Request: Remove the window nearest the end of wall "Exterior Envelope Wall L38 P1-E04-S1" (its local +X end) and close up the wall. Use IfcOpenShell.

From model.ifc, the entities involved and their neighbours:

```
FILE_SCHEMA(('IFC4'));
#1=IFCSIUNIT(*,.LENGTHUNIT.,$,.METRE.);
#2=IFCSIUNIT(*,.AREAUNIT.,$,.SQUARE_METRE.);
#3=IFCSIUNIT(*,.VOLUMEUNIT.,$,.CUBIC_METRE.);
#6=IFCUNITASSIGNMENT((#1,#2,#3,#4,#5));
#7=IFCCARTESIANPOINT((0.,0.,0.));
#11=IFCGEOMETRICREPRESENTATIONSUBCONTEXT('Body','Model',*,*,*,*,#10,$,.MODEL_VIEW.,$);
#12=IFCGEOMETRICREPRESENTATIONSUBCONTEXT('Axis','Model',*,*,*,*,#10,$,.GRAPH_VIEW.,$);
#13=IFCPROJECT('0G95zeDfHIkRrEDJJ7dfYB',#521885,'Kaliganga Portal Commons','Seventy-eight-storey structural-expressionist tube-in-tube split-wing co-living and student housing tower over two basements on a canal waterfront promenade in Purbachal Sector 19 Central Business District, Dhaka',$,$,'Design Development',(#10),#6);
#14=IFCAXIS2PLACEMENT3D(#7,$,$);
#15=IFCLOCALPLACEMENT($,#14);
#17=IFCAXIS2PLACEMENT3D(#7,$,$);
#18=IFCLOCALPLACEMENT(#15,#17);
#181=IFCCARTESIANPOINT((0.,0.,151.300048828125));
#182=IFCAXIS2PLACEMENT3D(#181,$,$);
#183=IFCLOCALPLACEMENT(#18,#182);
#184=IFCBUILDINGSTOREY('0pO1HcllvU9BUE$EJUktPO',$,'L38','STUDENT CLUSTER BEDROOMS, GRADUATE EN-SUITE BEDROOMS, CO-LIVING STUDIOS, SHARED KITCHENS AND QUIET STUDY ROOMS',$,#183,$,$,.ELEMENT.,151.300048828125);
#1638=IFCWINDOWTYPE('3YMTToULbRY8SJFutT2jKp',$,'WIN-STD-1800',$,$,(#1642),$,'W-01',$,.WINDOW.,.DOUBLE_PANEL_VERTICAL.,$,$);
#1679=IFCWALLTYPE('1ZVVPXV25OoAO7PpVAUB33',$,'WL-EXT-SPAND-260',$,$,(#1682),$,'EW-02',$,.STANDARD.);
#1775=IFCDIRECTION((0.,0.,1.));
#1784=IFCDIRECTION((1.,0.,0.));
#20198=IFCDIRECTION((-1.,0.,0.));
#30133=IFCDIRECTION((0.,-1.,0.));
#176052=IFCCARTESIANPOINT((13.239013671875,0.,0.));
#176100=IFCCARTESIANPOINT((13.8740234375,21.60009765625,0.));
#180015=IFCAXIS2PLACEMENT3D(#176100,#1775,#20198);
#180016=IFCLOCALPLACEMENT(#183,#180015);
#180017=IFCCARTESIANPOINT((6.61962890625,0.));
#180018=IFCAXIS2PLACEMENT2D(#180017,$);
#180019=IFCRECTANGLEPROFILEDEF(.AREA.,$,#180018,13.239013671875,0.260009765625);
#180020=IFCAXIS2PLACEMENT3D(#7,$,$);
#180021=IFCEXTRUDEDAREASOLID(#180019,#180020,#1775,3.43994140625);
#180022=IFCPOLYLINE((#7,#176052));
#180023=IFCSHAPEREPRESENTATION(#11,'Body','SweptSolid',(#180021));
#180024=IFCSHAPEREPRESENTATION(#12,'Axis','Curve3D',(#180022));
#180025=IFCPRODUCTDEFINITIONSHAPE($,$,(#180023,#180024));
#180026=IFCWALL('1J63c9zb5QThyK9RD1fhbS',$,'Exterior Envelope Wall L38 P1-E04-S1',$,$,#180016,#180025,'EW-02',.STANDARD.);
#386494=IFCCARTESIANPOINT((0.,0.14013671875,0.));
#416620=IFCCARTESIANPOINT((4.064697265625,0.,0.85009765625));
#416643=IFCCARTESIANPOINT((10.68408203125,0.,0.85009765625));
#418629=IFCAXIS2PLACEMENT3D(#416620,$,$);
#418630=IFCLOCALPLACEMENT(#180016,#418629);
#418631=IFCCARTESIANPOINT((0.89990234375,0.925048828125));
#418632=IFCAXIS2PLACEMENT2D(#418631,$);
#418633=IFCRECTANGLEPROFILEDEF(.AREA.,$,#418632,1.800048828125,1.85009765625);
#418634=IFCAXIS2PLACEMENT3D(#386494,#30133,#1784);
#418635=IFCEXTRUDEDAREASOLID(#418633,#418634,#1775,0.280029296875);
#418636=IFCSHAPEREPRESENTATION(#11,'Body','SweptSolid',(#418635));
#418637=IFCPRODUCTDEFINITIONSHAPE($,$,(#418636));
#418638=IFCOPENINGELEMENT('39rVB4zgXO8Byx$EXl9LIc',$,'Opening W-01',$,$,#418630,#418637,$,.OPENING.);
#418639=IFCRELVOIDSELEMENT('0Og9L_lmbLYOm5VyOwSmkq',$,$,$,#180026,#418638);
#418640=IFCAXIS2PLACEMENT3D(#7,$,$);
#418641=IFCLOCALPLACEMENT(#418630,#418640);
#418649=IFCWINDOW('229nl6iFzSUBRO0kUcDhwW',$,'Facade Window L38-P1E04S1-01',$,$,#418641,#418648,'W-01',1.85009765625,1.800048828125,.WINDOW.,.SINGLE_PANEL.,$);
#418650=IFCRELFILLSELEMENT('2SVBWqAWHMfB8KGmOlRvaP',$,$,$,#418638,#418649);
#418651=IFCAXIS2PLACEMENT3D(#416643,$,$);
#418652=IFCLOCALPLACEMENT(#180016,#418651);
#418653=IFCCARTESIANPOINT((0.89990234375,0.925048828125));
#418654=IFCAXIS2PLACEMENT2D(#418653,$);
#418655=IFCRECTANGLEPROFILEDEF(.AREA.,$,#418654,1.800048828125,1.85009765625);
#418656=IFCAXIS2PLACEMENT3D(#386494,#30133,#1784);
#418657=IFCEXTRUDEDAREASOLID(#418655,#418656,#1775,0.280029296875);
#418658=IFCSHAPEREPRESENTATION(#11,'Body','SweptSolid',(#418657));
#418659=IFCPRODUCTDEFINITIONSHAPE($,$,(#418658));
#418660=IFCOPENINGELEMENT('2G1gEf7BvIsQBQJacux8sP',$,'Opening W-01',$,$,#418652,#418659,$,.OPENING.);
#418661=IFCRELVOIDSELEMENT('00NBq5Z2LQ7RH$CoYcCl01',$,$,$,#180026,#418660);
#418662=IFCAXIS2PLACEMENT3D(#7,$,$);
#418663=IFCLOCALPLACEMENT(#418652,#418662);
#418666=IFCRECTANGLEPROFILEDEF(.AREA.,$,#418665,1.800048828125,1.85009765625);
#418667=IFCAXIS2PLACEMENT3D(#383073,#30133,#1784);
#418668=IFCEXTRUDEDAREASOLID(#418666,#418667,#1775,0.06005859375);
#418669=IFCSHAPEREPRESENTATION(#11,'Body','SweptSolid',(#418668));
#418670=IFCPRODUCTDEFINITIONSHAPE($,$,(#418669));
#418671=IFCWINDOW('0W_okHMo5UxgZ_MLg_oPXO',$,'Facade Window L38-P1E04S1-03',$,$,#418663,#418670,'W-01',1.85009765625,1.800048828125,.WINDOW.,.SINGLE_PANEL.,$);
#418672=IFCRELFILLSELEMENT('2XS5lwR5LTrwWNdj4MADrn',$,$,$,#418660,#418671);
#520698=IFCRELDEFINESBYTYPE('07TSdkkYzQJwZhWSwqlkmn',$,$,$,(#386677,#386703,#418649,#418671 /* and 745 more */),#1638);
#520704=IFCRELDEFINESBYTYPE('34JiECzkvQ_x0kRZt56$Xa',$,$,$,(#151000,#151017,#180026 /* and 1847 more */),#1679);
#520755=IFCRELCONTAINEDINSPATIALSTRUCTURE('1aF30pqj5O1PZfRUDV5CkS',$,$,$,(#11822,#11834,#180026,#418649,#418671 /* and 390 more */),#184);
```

```python
import ifcopenshell
import ifcopenshell.api.feature
import ifcopenshell.api.root
import ifcopenshell.geom
import ifcopenshell.util.shape

model = ifcopenshell.open("model.ifc")
settings = ifcopenshell.geom.settings()


def volume(element):
    """Net volume in cubic metres, openings subtracted."""
    shape = ifcopenshell.geom.create_shape(settings, element)
    return ifcopenshell.util.shape.get_volume(shape.geometry)


window = model.by_id(418671)
opening = window.FillsVoids[0].RelatingOpeningElement
wall = opening.VoidsElements[0].RelatingBuildingElement
before = volume(wall)

ifcopenshell.api.root.remove_product(model, product=window)
ifcopenshell.api.feature.remove_feature(model, feature=opening)

after = volume(wall)

print(f"wall volume {before:.3f} -> {after:.3f} m3")

model.write("model_v2.ifc")
```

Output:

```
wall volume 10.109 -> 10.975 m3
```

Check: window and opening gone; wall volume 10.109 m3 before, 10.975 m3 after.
